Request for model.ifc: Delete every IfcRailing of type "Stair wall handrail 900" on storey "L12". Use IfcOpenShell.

First a look at what the model holds.

```python
import ifcopenshell
import ifcopenshell.util.element

model = ifcopenshell.open("model.ifc")
print(model.schema)
storey = next(s for s in model.by_type("IfcBuildingStorey") if s.Name == "L12")
railings = [e for e in ifcopenshell.util.element.get_decomposition(storey) if e.is_a("IfcRailing")]
seen = {}
for e in railings:
    element_type = ifcopenshell.util.element.get_type(e)
    name = element_type.Name if element_type not in (None, e) else None
    seen[name] = seen.get(name, 0) + 1
for name, count in sorted(seen.items(), key=str):
    print(count, "x", name)
```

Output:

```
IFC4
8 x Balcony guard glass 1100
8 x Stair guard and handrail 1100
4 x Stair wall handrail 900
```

```python
import ifcopenshell
import ifcopenshell.api.root
import ifcopenshell.util.element

model = ifcopenshell.open("model.ifc")

storey = next(s for s in model.by_type("IfcBuildingStorey") if s.Name == "L12")
railings = [e for e in ifcopenshell.util.element.get_decomposition(storey) if e.is_a("IfcRailing")]
targets = [e for e in railings if (t := ifcopenshell.util.element.get_type(e)) not in (None, e) and t.Name == "Stair wall handrail 900"]

for e in targets:
    ifcopenshell.api.root.remove_product(model, product=e)
print(len(targets), "removed")

model.write("model_rev.ifc")
```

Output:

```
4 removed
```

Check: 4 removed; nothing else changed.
